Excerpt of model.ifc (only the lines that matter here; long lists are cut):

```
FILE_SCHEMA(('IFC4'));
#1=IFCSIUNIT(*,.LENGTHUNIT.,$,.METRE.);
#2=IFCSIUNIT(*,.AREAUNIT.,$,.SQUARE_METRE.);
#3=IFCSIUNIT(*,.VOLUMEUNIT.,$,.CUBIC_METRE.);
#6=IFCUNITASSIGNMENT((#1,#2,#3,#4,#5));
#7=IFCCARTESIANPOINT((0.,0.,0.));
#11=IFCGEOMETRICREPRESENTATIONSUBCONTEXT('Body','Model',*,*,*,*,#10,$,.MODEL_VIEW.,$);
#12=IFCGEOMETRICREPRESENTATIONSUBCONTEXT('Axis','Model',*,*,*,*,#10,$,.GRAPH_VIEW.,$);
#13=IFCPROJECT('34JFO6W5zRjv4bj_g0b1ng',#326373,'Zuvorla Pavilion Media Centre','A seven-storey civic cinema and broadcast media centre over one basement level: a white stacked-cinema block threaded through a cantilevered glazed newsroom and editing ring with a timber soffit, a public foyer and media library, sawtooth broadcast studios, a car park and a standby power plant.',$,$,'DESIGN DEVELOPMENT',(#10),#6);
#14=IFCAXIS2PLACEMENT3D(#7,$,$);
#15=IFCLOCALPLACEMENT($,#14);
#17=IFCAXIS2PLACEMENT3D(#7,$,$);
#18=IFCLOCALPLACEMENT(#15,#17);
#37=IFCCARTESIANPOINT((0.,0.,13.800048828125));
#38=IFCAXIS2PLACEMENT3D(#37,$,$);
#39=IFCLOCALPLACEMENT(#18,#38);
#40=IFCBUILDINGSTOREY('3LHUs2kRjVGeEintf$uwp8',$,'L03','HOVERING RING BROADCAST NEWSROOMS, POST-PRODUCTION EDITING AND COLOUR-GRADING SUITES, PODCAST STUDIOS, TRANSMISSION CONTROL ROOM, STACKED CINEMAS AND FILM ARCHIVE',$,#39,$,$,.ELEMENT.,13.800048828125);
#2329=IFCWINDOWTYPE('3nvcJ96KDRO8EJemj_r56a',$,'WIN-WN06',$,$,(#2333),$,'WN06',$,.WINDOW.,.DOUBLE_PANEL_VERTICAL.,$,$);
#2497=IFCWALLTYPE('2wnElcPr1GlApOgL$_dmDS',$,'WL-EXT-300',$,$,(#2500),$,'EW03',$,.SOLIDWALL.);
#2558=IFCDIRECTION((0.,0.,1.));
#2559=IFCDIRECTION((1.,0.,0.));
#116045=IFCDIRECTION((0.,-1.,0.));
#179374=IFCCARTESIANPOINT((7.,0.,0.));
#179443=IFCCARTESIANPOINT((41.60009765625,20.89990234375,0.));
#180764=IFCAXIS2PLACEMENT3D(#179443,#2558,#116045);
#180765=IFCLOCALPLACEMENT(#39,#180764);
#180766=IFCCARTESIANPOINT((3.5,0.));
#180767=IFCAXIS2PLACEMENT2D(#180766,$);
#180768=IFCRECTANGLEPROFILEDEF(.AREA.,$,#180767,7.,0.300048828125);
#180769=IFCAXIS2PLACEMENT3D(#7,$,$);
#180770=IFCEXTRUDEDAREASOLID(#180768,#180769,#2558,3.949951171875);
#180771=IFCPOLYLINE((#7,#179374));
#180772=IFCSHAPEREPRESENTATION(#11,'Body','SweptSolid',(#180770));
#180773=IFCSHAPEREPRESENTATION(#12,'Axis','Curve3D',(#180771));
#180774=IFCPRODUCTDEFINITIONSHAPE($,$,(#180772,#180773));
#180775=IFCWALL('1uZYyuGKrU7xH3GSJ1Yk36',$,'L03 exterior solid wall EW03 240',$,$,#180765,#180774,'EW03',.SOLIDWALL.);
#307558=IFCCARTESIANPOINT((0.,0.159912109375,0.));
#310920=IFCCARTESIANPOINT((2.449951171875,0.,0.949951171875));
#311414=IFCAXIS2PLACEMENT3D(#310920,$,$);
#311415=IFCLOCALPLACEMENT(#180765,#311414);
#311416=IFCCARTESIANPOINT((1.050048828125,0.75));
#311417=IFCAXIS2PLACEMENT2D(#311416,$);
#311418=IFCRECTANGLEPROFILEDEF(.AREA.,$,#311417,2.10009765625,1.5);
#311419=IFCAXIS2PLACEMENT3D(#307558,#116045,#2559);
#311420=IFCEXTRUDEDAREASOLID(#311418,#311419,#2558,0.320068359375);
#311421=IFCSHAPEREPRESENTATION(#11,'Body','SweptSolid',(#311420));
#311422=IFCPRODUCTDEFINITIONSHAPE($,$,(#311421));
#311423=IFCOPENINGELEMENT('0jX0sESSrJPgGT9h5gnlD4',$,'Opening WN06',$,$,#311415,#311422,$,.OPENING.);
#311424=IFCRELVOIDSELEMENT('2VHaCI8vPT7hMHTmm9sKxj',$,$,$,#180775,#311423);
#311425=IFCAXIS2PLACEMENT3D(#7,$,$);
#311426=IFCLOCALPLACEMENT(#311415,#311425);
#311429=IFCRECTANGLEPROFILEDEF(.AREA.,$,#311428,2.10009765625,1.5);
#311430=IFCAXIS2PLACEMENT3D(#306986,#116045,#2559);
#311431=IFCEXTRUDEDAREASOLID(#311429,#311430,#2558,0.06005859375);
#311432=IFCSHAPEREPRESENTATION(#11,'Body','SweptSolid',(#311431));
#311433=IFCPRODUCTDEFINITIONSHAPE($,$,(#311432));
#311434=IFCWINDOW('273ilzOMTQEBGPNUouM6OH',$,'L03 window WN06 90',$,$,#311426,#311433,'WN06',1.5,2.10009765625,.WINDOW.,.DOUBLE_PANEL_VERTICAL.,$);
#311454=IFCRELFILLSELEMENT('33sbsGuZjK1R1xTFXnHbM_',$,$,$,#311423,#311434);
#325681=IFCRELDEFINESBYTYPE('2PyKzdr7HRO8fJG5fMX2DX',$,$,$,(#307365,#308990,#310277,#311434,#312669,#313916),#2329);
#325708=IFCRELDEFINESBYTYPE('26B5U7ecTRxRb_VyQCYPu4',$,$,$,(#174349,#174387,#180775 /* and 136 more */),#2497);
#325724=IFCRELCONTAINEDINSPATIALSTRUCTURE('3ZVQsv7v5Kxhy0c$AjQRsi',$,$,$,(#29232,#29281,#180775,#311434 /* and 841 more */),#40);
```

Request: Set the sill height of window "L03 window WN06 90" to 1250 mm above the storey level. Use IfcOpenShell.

```python
import numpy as np
import ifcopenshell
import ifcopenshell.api.geometry
import ifcopenshell.geom
import ifcopenshell.util.element
import ifcopenshell.util.placement
import ifcopenshell.util.shape
import ifcopenshell.util.unit

model = ifcopenshell.open("model.ifc")
unit_scale = ifcopenshell.util.unit.calculate_unit_scale(model)

window = model.by_id(311434)
opening = window.FillsVoids[0].RelatingOpeningElement
storey = ifcopenshell.util.element.get_container(window, ifc_class="IfcBuildingStorey")
level = ifcopenshell.util.placement.get_local_placement(storey.ObjectPlacement)[2, 3]

# The opening's origin need not be at the sill, so measure its lowest point.
shape = ifcopenshell.geom.create_shape(ifcopenshell.geom.settings(), opening)
bottom = ifcopenshell.util.shape.get_shape_bottom_elevation(shape, shape.geometry) / unit_scale
dz = level + 1.25 / unit_scale - bottom

shift = np.array([0.0, 0.0, dz])
# The window is placed relative to its opening, so it follows when the opening moves.
matrix = ifcopenshell.util.placement.get_local_placement(opening.ObjectPlacement)
matrix[:3, 3] += shift
ifcopenshell.api.geometry.edit_object_placement(
    model, product=opening, matrix=matrix, is_si=False, should_transform_children=True
)

print(f"moved by {dz * unit_scale:+.3f} m")

model.write("model-out.ifc")
```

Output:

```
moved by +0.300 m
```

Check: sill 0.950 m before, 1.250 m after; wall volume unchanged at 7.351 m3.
